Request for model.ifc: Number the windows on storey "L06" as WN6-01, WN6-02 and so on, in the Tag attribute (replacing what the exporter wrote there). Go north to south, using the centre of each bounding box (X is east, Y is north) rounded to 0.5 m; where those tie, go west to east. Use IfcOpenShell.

First a look at what the model holds.

```python
import ifcopenshell
import ifcopenshell.util.element
import ifcopenshell.util.placement

model = ifcopenshell.open("model.ifc")
print(model.schema)
storey = next(s for s in model.by_type("IfcBuildingStorey") if s.Name == "L06")
windows = [e for e in ifcopenshell.util.element.get_decomposition(storey) if e.is_a("IfcWindow")]
for e in sorted(windows, key=lambda e: e.id()):
    origin = ifcopenshell.util.placement.get_local_placement(e.ObjectPlacement)[:3, 3]
    print(e.id(), e.Tag, e.Name, origin.round(2) + 0.0, sep=" | ")
```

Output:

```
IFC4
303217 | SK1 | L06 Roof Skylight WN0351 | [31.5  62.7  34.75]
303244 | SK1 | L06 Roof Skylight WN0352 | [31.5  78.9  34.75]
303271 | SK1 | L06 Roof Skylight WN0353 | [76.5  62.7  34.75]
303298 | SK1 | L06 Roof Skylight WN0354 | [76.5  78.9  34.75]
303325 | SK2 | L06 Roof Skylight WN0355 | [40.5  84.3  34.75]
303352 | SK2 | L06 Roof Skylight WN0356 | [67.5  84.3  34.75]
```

```python
import ifcopenshell
import ifcopenshell.geom
import ifcopenshell.util.element
import ifcopenshell.util.shape

model = ifcopenshell.open("model.ifc")
settings = ifcopenshell.geom.settings()
settings.set("use-world-coords", True)


def centre(element):
    shape = ifcopenshell.geom.create_shape(settings, element)
    return ifcopenshell.util.shape.get_bbox_centroid(shape.geometry)


storey = next(s for s in model.by_type("IfcBuildingStorey") if s.Name == "L06")
windows = [e for e in ifcopenshell.util.element.get_decomposition(storey) if e.is_a("IfcWindow")]

# Insertion points can sit at a corner or the storey origin, so sort by the geometry (in metres).
centres = {e: centre(e) for e in windows}
windows.sort(key=lambda e: (-round(centres[e][1] / 0.5), centres[e][0]))

for i, e in enumerate(windows, start=1):
    number = f"WN6-{i:02d}"
    e.Tag = number
    print(e.id(), number)

model.write("model_updated.ifc")
```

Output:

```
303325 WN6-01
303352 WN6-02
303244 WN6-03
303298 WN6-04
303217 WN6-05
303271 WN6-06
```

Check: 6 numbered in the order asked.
